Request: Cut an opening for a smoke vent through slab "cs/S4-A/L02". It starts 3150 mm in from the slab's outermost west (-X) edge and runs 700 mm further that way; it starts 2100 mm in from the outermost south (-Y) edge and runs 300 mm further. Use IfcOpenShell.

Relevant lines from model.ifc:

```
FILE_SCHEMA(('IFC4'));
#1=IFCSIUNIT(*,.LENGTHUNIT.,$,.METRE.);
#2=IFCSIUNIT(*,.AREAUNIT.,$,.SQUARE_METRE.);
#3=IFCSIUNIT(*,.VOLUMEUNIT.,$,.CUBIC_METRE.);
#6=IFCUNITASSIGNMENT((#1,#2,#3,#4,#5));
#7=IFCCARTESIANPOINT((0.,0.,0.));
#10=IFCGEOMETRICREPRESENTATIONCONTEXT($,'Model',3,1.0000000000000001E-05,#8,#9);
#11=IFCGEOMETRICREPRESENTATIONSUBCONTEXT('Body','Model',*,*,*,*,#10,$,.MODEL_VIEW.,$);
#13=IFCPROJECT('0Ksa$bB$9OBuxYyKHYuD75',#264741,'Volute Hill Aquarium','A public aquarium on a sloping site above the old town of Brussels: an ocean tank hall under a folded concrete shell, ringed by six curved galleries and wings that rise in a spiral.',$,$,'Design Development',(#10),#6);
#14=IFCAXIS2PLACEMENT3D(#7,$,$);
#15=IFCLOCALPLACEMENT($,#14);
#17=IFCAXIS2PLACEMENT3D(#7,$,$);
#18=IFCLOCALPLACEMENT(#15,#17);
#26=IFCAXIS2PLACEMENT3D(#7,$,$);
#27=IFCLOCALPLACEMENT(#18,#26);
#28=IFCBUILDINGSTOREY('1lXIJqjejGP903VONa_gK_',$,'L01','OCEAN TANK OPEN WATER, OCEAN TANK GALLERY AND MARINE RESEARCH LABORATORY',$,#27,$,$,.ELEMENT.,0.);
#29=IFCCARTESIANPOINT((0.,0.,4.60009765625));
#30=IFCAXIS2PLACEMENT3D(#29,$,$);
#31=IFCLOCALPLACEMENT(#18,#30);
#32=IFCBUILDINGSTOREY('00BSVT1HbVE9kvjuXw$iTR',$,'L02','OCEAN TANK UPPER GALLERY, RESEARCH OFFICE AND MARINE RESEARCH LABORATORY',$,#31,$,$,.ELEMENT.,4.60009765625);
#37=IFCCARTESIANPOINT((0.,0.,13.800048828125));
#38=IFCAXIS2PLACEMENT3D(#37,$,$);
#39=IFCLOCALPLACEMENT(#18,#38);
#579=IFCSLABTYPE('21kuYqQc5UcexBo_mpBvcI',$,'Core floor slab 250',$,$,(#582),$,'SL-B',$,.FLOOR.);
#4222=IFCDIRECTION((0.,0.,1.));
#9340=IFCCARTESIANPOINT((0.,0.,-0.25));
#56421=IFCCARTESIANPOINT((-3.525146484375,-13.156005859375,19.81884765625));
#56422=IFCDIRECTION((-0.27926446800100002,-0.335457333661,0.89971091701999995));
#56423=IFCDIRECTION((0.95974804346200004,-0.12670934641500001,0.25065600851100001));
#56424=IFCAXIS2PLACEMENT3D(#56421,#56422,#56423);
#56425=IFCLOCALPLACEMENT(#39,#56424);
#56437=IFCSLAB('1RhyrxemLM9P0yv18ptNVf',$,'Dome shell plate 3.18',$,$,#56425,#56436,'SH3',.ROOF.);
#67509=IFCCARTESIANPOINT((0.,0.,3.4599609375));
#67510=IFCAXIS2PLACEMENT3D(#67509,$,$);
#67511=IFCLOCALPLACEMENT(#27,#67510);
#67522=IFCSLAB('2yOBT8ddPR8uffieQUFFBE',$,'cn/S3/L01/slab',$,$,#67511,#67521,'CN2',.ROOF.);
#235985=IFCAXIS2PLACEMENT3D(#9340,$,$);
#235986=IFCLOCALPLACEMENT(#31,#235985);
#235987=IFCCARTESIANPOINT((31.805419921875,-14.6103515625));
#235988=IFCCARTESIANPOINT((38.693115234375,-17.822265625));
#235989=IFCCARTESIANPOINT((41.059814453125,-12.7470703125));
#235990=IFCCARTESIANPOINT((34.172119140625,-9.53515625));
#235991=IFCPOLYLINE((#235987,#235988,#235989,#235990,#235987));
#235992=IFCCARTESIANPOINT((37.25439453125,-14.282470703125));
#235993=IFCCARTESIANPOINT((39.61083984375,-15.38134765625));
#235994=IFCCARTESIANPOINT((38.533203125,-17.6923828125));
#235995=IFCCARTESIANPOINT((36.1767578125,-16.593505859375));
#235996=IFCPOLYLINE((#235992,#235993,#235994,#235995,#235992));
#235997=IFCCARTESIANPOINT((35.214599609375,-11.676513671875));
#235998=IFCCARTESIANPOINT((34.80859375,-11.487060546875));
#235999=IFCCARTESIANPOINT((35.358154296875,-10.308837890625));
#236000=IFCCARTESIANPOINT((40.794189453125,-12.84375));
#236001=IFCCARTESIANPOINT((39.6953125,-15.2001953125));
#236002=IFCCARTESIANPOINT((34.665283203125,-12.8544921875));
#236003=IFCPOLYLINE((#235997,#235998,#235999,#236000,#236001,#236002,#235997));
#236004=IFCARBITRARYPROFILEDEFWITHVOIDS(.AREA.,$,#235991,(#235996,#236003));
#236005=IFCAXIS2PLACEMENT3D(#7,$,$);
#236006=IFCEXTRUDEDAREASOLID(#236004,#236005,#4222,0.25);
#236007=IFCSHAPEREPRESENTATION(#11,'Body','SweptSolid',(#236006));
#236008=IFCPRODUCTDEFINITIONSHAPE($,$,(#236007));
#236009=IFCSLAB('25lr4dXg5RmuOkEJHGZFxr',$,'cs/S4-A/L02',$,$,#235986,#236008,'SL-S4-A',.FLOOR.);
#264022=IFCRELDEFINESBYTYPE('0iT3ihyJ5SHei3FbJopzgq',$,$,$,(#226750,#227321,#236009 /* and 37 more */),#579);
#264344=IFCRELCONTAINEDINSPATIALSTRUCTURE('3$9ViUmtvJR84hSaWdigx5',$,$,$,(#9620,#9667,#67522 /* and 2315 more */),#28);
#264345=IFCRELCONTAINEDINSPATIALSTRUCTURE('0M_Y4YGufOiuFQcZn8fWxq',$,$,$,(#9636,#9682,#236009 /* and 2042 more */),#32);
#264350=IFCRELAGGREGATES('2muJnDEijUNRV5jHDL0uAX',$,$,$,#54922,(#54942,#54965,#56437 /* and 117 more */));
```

```python
import numpy as np
import ifcopenshell
import ifcopenshell.api.feature
import ifcopenshell.api.geometry
import ifcopenshell.api.root
import ifcopenshell.geom
import ifcopenshell.util.placement
import ifcopenshell.util.representation
import ifcopenshell.util.shape
import ifcopenshell.util.unit

model = ifcopenshell.open("model.ifc")
unit_scale = ifcopenshell.util.unit.calculate_unit_scale(model)
settings = ifcopenshell.geom.settings()


def volume(element):
    """Net volume in cubic metres, openings subtracted."""
    shape = ifcopenshell.geom.create_shape(settings, element)
    return ifcopenshell.util.shape.get_volume(shape.geometry)


slab = model.by_guid("25lr4dXg5RmuOkEJHGZFxr")
before = volume(slab)

# Extent in the slab's own axes, in metres. The edges named are its -X and -Y sides.
slab_shape = ifcopenshell.geom.create_shape(settings, slab)
vertices = ifcopenshell.util.shape.get_vertices(slab_shape.geometry)
x_min, y_min, bottom = vertices.min(axis=0)
top = vertices[:, 2].max()

opening = ifcopenshell.api.root.create_entity(model, ifc_class="IfcOpeningElement", name="Smoke vent opening", predefined_type="OPENING")
context = ifcopenshell.util.representation.get_context(model, "Model", "Body", "MODEL_VIEW")
width, depth = 0.7, 0.3
outline = [(0.0, 0.0), (width, 0.0), (width, depth), (0.0, depth), (0.0, 0.0)]
# Overshoot both faces by 50 mm so the cut is clean.
shape = ifcopenshell.api.geometry.add_slab_representation(
    model, context=context, depth=top - bottom + 0.1, polyline=outline
)
ifcopenshell.api.geometry.assign_representation(model, product=opening, representation=shape)

matrix = ifcopenshell.util.placement.get_local_placement(slab.ObjectPlacement)
matrix[:, 3] = matrix @ np.append(np.array([x_min + 3.15, y_min + 2.1, bottom - 0.05]) / unit_scale, 1.0)
ifcopenshell.api.geometry.edit_object_placement(model, product=opening, matrix=matrix, is_si=False)
ifcopenshell.api.feature.add_feature(model, feature=opening, element=slab)

after = volume(slab)

print(f"slab volume {before:.3f} -> {after:.3f} m3")

model.write("model_v2.ifc")
```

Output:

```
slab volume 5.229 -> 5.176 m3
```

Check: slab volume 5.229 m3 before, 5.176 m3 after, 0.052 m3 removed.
